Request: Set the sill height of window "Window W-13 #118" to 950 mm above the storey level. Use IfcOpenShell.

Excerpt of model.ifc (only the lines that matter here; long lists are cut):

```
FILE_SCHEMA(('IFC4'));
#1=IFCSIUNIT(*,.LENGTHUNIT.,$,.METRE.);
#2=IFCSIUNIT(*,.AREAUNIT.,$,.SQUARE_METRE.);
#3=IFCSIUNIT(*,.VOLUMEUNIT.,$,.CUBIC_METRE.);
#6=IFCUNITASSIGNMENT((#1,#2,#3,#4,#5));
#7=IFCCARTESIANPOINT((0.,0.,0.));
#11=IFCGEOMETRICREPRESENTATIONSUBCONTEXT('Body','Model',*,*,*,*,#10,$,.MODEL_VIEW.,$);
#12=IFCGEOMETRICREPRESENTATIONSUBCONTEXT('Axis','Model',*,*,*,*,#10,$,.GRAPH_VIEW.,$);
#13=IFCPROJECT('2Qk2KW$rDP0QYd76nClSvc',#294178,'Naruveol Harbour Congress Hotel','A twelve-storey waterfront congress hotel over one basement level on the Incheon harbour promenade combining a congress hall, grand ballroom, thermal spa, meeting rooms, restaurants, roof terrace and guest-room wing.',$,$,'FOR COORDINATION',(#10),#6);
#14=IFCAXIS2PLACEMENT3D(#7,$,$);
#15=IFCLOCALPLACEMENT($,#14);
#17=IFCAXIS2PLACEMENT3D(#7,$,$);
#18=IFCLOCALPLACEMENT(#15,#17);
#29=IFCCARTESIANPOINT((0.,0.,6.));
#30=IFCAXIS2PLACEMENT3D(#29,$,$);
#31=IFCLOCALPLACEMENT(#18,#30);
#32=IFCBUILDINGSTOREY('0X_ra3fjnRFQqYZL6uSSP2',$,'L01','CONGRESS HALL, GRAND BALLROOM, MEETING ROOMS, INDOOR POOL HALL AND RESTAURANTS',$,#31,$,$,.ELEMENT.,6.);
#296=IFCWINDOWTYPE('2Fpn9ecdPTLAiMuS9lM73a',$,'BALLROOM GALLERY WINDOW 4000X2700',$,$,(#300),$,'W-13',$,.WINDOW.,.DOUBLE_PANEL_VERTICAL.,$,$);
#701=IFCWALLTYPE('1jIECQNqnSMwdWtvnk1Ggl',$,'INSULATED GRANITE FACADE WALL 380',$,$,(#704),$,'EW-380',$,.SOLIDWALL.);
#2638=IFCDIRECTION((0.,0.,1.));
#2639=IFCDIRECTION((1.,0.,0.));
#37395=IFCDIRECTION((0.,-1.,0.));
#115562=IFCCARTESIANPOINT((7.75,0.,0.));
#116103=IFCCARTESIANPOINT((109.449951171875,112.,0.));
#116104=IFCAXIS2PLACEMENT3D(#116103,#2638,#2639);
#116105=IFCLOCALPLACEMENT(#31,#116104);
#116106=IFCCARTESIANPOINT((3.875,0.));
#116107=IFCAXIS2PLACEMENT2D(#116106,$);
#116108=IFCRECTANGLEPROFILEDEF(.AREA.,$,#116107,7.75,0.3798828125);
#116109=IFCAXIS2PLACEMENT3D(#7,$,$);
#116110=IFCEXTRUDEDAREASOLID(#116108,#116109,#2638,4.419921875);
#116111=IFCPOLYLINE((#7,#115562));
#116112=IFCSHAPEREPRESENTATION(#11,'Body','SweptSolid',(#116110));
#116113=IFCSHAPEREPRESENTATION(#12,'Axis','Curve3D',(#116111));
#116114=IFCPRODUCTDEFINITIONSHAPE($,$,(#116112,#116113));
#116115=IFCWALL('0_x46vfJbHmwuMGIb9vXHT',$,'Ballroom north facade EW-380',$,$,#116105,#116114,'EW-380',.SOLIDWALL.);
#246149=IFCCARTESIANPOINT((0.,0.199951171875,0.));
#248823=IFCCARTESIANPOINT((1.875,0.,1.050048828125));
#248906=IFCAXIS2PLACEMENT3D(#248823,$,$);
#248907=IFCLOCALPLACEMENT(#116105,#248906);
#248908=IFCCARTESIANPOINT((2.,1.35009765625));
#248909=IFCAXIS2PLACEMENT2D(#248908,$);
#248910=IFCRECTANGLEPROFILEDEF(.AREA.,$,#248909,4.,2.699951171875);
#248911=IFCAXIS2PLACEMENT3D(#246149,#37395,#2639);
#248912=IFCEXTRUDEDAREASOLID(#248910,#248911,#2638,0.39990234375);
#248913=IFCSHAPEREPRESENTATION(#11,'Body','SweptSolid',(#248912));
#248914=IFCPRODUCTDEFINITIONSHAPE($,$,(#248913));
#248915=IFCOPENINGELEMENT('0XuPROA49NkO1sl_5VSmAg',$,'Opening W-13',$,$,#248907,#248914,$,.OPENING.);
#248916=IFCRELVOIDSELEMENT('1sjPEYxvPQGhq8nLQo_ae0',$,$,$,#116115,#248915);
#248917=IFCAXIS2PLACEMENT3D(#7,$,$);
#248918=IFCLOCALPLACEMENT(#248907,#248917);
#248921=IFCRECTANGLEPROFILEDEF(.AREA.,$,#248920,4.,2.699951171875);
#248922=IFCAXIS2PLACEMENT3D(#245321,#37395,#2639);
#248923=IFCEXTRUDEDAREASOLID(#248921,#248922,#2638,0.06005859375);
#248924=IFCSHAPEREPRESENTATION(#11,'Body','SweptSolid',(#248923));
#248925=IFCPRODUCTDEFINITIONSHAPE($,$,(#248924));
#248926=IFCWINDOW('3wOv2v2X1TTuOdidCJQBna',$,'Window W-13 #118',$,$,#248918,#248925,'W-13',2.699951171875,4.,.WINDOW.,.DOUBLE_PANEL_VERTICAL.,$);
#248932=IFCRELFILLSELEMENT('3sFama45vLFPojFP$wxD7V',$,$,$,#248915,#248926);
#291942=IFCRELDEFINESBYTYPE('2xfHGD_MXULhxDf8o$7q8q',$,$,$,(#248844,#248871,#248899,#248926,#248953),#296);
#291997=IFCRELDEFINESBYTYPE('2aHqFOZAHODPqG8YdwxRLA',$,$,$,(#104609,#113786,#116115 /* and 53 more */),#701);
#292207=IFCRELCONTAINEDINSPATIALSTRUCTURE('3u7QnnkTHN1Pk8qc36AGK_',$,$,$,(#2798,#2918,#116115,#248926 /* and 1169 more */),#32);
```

```python
import numpy as np
import ifcopenshell
import ifcopenshell.api.geometry
import ifcopenshell.geom
import ifcopenshell.util.element
import ifcopenshell.util.placement
import ifcopenshell.util.shape
import ifcopenshell.util.unit

model = ifcopenshell.open("model.ifc")
unit_scale = ifcopenshell.util.unit.calculate_unit_scale(model)

window = model.by_guid("3wOv2v2X1TTuOdidCJQBna")
opening = window.FillsVoids[0].RelatingOpeningElement
storey = ifcopenshell.util.element.get_container(window, ifc_class="IfcBuildingStorey")
level = ifcopenshell.util.placement.get_local_placement(storey.ObjectPlacement)[2, 3]

# The opening's origin need not be at the sill, so measure its lowest point.
shape = ifcopenshell.geom.create_shape(ifcopenshell.geom.settings(), opening)
bottom = ifcopenshell.util.shape.get_shape_bottom_elevation(shape, shape.geometry) / unit_scale
dz = level + 0.95 / unit_scale - bottom

shift = np.array([0.0, 0.0, dz])
# The window is placed relative to its opening, so it follows when the opening moves.
matrix = ifcopenshell.util.placement.get_local_placement(opening.ObjectPlacement)
matrix[:3, 3] += shift
ifcopenshell.api.geometry.edit_object_placement(
    model, product=opening, matrix=matrix, is_si=False, should_transform_children=True
)

print(f"moved by {dz * unit_scale:+.3f} m")

model.write("model_rev.ifc")
```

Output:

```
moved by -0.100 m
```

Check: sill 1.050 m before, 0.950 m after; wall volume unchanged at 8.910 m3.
